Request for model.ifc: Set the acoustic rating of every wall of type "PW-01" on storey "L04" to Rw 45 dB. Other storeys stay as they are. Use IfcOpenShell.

First a look at what the model holds.

```python
import ifcopenshell
import ifcopenshell.util.element

model = ifcopenshell.open("model.ifc")
print(model.schema)
storey = next(s for s in model.by_type("IfcBuildingStorey") if s.Name == "L04")
walls = [e for e in ifcopenshell.util.element.get_decomposition(storey) if e.is_a("IfcWall")]
seen = {}
for e in walls:
    element_type = ifcopenshell.util.element.get_type(e)
    key = (element_type.Name if element_type != e and element_type else None, ifcopenshell.util.element.get_pset(e, "Pset_WallCommon", "AcousticRating"))
    seen[key] = seen.get(key, 0) + 1
for (name, value), count in sorted(seen.items(), key=str):
    print(count, "x", name, "|", value)
```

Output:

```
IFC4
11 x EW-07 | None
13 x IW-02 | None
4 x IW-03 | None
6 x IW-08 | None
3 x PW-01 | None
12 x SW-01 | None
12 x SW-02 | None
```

```python
import ifcopenshell
import ifcopenshell.api.pset
import ifcopenshell.util.element

model = ifcopenshell.open("model.ifc")

storey = next(s for s in model.by_type("IfcBuildingStorey") if s.Name == "L04")
walls = [e for e in ifcopenshell.util.element.get_decomposition(storey) if e.is_a("IfcWall")]

count = 0
for e in walls:
    element_type = ifcopenshell.util.element.get_type(e)
    if element_type in (None, e) or element_type.Name != "PW-01":
        continue
    # add_pset returns the element's existing set when there is one.
    pset = ifcopenshell.api.pset.add_pset(model, product=e, name="Pset_WallCommon")
    ifcopenshell.api.pset.edit_pset(model, pset=pset, properties={"AcousticRating": "Rw 45 dB"})
    count += 1

print(count, "walls updated")

model.write("model_rev.ifc")
```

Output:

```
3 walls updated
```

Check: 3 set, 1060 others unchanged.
